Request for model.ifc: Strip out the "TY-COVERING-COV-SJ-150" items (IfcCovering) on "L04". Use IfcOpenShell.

First a look at what the model holds.

```python
import ifcopenshell
import ifcopenshell.util.element

model = ifcopenshell.open("model.ifc")
print(model.schema)
storey = next(s for s in model.by_type("IfcBuildingStorey") if s.Name == "L04")
coverings = [e for e in ifcopenshell.util.element.get_decomposition(storey) if e.is_a("IfcCovering")]
seen = {}
for e in coverings:
    element_type = ifcopenshell.util.element.get_type(e)
    name = element_type.Name if element_type not in (None, e) else None
    seen[name] = seen.get(name, 0) + 1
for name, count in sorted(seen.items(), key=str):
    print(count, "x", name)
```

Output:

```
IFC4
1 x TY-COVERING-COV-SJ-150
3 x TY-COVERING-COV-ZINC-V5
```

```python
import ifcopenshell
import ifcopenshell.api.root
import ifcopenshell.util.element

model = ifcopenshell.open("model.ifc")

storey = next(s for s in model.by_type("IfcBuildingStorey") if s.Name == "L04")
coverings = [e for e in ifcopenshell.util.element.get_decomposition(storey) if e.is_a("IfcCovering")]
targets = [e for e in coverings if (t := ifcopenshell.util.element.get_type(e)) not in (None, e) and t.Name == "TY-COVERING-COV-SJ-150"]

for e in targets:
    ifcopenshell.api.root.remove_product(model, product=e)
print(len(targets), "removed")

model.write("model_rev.ifc")
```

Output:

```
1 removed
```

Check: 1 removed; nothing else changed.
